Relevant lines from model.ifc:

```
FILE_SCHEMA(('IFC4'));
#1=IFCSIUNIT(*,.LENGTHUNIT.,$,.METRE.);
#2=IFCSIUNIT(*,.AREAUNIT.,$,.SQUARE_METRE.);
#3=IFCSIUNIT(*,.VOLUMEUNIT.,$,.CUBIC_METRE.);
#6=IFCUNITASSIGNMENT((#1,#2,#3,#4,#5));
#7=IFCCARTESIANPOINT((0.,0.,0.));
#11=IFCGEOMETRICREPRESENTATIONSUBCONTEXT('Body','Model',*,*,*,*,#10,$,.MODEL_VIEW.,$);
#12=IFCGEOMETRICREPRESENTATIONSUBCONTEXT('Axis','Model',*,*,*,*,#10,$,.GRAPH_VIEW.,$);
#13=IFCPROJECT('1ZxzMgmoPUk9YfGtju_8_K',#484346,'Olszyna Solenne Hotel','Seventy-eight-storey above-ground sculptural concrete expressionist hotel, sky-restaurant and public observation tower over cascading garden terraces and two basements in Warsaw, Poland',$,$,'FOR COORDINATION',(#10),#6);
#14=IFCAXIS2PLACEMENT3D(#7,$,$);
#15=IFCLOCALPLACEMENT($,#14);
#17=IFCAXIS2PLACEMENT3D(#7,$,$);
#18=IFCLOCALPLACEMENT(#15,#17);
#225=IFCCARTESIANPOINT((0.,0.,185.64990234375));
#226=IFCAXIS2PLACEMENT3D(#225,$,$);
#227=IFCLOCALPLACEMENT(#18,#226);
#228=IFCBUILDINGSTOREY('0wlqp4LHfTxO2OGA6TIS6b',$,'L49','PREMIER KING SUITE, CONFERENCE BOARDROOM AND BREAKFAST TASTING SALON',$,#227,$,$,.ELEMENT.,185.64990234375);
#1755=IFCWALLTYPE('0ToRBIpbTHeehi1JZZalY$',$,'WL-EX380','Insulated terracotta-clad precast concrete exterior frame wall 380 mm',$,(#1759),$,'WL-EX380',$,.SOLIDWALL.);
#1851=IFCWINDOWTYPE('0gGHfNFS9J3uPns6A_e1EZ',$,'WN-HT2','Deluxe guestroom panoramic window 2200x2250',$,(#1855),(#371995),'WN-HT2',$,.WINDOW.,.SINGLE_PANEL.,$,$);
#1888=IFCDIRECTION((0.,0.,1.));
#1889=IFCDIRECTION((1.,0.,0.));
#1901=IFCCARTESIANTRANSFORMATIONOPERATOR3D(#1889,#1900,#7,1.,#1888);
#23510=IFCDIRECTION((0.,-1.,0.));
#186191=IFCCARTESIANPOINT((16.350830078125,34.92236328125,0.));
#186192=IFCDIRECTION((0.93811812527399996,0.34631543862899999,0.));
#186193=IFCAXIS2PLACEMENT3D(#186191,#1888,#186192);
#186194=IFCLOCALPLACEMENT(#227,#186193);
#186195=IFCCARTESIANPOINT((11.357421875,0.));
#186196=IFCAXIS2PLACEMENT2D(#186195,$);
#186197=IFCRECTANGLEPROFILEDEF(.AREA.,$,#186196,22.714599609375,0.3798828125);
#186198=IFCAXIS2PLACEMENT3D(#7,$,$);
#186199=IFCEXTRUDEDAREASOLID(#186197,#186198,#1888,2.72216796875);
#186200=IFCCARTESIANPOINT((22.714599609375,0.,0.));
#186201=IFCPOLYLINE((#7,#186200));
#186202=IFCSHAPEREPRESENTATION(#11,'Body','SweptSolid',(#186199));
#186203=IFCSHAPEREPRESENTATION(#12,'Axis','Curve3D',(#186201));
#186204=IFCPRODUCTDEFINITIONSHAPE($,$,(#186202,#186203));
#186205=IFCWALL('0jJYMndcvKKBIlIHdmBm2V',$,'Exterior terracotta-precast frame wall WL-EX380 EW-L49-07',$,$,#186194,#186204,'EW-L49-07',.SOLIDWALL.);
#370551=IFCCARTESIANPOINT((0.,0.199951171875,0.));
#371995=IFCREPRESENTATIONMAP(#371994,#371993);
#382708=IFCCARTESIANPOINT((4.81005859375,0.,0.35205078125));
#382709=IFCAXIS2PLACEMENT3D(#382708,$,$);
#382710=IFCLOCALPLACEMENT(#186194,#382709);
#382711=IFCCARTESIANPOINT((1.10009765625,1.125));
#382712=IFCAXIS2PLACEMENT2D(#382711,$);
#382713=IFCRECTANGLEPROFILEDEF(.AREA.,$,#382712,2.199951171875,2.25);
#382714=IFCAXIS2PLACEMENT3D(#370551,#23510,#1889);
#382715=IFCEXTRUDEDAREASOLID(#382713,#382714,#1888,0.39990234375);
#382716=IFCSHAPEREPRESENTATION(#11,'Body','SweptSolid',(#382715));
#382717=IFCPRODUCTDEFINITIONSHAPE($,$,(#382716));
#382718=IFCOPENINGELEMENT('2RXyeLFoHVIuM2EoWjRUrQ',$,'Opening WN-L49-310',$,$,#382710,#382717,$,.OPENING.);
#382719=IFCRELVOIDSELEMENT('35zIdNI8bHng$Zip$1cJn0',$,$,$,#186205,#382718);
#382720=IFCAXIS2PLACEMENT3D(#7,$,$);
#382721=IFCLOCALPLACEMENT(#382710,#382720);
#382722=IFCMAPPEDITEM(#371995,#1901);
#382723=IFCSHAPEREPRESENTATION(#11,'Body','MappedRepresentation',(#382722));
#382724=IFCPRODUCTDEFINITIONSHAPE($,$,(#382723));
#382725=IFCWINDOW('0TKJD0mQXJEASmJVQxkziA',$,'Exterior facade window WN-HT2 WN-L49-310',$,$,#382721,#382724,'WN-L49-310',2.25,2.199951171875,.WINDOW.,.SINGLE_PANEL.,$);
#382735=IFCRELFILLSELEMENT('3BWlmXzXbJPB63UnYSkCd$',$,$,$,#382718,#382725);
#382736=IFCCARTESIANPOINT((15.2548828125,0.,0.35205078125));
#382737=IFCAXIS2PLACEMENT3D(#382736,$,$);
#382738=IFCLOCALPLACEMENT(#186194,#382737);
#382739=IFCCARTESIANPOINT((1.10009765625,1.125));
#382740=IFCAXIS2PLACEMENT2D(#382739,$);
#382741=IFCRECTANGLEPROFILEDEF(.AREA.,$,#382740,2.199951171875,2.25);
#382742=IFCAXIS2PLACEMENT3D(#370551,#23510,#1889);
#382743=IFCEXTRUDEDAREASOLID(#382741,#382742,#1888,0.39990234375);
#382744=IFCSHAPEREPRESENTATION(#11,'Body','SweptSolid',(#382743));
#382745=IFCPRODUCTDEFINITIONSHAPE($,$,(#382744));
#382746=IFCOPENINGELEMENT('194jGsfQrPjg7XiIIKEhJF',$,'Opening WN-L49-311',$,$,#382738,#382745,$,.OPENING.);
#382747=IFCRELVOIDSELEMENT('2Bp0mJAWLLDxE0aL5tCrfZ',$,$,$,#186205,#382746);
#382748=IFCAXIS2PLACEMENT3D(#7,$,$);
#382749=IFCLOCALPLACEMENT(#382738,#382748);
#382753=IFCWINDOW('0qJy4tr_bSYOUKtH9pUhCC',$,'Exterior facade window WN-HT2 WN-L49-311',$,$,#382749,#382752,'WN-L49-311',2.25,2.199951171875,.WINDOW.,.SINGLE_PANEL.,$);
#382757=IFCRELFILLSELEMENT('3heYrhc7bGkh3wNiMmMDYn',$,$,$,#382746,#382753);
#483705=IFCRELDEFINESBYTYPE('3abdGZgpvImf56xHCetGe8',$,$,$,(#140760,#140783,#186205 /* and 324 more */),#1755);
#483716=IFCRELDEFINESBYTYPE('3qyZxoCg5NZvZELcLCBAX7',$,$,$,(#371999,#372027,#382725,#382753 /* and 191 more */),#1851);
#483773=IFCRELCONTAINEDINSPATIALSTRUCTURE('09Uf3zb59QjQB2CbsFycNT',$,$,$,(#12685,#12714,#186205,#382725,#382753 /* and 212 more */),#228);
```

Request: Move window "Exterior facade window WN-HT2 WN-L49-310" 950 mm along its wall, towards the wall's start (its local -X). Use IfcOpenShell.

```python
import ifcopenshell
import ifcopenshell.api.geometry
import ifcopenshell.util.placement
import ifcopenshell.util.unit

model = ifcopenshell.open("model.ifc")
unit_scale = ifcopenshell.util.unit.calculate_unit_scale(model)

window = model.by_guid("0TKJD0mQXJEASmJVQxkziA")
opening = window.FillsVoids[0].RelatingOpeningElement
wall = opening.VoidsElements[0].RelatingBuildingElement

wall_matrix = ifcopenshell.util.placement.get_local_placement(wall.ObjectPlacement)
shift = wall_matrix[:3, 0] * -0.95 / unit_scale
before = ifcopenshell.util.placement.get_local_placement(window.ObjectPlacement)[:3, 3].copy()

# The window is placed relative to its opening, so it follows when the opening moves.
matrix = ifcopenshell.util.placement.get_local_placement(opening.ObjectPlacement)
matrix[:3, 3] += shift
ifcopenshell.api.geometry.edit_object_placement(
    model, product=opening, matrix=matrix, is_si=False, should_transform_children=True
)

after = ifcopenshell.util.placement.get_local_placement(window.ObjectPlacement)[:3, 3]
print("window moved by", (after - before).round(3) + 0.0)

model.write("model-out.ifc")
```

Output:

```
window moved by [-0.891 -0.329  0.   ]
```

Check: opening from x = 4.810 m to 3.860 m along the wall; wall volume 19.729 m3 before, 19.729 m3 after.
